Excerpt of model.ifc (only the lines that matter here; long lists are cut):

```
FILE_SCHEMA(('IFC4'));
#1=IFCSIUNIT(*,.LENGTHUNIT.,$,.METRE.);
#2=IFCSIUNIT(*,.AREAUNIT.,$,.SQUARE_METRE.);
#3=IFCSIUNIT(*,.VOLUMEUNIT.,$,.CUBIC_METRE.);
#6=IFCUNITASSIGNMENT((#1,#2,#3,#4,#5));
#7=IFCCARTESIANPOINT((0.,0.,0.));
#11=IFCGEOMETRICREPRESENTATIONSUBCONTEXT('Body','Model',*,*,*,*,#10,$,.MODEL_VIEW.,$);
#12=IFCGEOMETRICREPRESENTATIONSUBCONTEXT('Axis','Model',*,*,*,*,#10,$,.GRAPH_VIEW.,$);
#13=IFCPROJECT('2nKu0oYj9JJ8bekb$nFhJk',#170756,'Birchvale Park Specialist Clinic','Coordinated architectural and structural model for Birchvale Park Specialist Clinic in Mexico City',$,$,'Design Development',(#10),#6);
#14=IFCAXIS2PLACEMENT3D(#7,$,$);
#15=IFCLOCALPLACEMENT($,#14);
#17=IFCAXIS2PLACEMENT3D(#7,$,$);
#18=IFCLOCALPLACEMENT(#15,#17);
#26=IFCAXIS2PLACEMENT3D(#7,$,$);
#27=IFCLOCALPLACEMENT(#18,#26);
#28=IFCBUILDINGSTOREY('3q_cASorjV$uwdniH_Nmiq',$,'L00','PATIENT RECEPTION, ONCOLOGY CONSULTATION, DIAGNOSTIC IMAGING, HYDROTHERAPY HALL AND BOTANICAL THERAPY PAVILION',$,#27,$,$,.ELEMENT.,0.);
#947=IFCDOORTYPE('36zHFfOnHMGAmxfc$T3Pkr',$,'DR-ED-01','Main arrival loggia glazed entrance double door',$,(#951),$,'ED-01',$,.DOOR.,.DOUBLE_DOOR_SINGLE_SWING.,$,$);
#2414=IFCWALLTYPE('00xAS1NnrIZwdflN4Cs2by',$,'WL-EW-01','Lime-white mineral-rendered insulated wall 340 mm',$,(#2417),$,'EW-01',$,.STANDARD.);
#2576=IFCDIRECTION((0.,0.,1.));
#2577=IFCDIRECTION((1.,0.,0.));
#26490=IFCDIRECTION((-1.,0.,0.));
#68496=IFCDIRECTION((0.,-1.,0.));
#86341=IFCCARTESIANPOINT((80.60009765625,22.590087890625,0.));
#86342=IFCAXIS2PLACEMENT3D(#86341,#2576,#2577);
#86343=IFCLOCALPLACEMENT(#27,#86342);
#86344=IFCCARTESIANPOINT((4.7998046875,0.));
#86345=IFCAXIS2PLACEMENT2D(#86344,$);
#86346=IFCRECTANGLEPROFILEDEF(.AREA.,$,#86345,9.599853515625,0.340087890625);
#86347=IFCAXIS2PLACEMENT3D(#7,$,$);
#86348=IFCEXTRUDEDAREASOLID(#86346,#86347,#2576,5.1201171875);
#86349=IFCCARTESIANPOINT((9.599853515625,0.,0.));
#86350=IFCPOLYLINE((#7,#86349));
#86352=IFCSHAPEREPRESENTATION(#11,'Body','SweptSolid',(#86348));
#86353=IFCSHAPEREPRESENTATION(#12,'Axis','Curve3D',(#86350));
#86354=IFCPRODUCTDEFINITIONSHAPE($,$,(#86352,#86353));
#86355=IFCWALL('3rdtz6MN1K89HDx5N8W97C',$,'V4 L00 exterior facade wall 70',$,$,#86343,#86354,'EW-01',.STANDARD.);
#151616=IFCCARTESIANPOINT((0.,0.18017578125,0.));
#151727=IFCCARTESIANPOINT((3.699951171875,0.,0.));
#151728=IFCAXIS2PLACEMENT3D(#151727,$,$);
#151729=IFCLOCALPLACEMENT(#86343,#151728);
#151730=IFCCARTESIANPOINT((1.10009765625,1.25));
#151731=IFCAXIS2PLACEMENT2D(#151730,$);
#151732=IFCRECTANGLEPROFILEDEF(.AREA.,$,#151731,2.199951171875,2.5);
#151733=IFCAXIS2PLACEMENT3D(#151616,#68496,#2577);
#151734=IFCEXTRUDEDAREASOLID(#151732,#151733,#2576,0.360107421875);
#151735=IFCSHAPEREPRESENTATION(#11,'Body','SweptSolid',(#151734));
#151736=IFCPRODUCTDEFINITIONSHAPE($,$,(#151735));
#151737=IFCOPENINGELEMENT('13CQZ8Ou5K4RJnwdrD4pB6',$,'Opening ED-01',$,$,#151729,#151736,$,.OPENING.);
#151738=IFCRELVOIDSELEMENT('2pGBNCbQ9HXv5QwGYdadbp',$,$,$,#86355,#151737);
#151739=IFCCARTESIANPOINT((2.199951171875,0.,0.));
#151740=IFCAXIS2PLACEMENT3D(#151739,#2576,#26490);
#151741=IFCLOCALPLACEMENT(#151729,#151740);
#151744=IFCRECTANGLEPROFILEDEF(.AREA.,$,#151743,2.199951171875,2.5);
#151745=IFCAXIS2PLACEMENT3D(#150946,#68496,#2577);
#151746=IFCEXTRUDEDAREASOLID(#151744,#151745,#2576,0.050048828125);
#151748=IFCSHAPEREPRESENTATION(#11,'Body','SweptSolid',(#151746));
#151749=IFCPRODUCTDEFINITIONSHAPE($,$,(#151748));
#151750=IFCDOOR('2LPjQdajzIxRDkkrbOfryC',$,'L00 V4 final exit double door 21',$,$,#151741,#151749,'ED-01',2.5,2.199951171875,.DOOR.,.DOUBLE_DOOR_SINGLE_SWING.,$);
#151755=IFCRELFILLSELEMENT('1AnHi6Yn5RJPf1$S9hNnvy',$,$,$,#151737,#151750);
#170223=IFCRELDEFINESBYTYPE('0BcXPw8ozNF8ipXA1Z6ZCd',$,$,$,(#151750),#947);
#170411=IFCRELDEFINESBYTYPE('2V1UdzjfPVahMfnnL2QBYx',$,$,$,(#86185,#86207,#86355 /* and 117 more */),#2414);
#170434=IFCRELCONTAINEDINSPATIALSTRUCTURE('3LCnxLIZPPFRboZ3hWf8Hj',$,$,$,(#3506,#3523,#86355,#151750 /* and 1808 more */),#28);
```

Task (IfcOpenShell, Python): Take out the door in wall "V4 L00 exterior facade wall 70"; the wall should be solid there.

```python
import ifcopenshell
import ifcopenshell.api.feature
import ifcopenshell.api.root
import ifcopenshell.geom
import ifcopenshell.util.shape

model = ifcopenshell.open("model.ifc")
settings = ifcopenshell.geom.settings()


def volume(element):
    """Net volume in cubic metres, openings subtracted."""
    shape = ifcopenshell.geom.create_shape(settings, element)
    return ifcopenshell.util.shape.get_volume(shape.geometry)


door = model.by_guid("2LPjQdajzIxRDkkrbOfryC")
opening = door.FillsVoids[0].RelatingOpeningElement
wall = opening.VoidsElements[0].RelatingBuildingElement
before = volume(wall)

ifcopenshell.api.root.remove_product(model, product=door)
ifcopenshell.api.feature.remove_feature(model, feature=opening)

after = volume(wall)

print(f"wall volume {before:.3f} -> {after:.3f} m3")

model.write("model-out.ifc")
```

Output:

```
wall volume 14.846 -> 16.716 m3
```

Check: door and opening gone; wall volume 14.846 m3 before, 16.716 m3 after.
